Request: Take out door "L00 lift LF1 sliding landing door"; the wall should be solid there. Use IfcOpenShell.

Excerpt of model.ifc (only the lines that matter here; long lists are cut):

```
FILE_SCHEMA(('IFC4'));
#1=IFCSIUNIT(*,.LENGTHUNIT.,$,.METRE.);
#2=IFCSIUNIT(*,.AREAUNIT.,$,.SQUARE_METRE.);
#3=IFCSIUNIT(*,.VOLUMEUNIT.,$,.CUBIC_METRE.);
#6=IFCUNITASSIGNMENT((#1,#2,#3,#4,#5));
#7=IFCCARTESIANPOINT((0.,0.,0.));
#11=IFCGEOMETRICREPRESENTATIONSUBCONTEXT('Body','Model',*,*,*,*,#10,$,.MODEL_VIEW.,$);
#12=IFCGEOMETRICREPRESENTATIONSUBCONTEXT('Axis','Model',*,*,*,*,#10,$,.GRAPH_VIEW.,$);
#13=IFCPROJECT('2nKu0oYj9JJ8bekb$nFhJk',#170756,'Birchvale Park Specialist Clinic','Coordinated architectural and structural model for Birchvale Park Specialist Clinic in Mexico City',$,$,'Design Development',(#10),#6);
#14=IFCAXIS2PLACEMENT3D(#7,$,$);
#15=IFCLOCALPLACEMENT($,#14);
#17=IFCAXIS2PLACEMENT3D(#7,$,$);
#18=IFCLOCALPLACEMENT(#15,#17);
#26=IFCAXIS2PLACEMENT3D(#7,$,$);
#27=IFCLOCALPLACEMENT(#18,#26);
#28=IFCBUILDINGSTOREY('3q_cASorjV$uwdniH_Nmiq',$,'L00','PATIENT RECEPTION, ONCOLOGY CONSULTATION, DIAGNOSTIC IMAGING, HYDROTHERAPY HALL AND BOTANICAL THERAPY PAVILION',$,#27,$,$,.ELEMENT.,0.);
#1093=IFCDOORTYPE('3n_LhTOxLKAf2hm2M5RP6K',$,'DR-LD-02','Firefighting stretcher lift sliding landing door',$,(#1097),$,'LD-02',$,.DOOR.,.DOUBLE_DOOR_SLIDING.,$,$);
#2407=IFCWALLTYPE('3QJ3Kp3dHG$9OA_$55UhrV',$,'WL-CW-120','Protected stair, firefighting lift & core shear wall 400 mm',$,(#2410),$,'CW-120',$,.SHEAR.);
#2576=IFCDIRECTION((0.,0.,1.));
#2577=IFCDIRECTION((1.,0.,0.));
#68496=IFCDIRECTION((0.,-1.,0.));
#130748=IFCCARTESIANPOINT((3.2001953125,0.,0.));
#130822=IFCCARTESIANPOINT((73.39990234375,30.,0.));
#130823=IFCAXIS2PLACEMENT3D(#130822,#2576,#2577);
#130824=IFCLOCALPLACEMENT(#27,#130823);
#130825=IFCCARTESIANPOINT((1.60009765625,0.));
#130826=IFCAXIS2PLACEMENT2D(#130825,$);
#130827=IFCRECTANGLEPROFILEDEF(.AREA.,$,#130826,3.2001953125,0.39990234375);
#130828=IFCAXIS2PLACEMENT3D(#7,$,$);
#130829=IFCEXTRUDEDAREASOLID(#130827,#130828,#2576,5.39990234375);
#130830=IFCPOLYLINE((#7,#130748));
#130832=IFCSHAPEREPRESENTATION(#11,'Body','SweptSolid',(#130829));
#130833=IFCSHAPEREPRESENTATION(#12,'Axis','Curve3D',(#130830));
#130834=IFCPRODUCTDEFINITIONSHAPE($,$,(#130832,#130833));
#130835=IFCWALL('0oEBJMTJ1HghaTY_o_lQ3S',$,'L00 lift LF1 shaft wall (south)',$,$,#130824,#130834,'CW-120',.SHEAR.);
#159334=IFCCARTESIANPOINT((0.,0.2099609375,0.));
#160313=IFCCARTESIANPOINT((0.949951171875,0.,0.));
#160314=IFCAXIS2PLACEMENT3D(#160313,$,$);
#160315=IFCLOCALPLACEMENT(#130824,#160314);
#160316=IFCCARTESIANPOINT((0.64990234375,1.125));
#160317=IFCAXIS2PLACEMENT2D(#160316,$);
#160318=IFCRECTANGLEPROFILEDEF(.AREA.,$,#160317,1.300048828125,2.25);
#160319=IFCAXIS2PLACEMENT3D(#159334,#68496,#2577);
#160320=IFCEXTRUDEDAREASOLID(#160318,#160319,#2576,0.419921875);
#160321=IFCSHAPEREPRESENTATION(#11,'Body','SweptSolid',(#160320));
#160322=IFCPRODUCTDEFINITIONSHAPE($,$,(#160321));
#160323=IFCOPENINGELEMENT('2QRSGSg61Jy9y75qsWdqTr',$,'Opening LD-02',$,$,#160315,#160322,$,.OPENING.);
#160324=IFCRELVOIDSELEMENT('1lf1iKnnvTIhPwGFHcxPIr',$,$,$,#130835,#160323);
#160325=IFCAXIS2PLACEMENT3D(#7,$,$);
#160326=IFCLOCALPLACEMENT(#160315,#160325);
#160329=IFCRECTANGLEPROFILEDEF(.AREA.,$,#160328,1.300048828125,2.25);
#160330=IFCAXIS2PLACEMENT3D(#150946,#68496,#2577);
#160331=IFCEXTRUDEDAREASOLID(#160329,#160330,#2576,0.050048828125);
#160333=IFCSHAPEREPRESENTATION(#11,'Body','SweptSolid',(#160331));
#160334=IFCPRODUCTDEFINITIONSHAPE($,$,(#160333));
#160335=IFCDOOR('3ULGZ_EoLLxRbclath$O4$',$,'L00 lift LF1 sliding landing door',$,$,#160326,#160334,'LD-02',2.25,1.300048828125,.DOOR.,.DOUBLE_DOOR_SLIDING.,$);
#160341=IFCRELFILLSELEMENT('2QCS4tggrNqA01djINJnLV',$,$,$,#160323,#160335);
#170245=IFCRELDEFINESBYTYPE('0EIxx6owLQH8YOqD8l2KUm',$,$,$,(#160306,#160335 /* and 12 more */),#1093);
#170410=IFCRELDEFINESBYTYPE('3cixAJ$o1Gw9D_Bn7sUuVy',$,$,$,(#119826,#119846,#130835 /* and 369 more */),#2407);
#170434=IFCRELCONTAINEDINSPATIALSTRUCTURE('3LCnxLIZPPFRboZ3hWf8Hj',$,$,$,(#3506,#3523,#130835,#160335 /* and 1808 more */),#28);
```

```python
import ifcopenshell
import ifcopenshell.api.feature
import ifcopenshell.api.root
import ifcopenshell.geom
import ifcopenshell.util.shape

model = ifcopenshell.open("model.ifc")
settings = ifcopenshell.geom.settings()


def volume(element):
    """Net volume in cubic metres, openings subtracted."""
    shape = ifcopenshell.geom.create_shape(settings, element)
    return ifcopenshell.util.shape.get_volume(shape.geometry)


door = model.by_guid("3ULGZ_EoLLxRbclath$O4$")
opening = door.FillsVoids[0].RelatingOpeningElement
wall = opening.VoidsElements[0].RelatingBuildingElement
before = volume(wall)

ifcopenshell.api.root.remove_product(model, product=door)
ifcopenshell.api.feature.remove_feature(model, feature=opening)

after = volume(wall)

print(f"wall volume {before:.3f} -> {after:.3f} m3")

model.write("model_edited.ifc")
```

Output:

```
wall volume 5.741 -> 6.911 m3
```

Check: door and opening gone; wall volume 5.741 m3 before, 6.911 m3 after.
